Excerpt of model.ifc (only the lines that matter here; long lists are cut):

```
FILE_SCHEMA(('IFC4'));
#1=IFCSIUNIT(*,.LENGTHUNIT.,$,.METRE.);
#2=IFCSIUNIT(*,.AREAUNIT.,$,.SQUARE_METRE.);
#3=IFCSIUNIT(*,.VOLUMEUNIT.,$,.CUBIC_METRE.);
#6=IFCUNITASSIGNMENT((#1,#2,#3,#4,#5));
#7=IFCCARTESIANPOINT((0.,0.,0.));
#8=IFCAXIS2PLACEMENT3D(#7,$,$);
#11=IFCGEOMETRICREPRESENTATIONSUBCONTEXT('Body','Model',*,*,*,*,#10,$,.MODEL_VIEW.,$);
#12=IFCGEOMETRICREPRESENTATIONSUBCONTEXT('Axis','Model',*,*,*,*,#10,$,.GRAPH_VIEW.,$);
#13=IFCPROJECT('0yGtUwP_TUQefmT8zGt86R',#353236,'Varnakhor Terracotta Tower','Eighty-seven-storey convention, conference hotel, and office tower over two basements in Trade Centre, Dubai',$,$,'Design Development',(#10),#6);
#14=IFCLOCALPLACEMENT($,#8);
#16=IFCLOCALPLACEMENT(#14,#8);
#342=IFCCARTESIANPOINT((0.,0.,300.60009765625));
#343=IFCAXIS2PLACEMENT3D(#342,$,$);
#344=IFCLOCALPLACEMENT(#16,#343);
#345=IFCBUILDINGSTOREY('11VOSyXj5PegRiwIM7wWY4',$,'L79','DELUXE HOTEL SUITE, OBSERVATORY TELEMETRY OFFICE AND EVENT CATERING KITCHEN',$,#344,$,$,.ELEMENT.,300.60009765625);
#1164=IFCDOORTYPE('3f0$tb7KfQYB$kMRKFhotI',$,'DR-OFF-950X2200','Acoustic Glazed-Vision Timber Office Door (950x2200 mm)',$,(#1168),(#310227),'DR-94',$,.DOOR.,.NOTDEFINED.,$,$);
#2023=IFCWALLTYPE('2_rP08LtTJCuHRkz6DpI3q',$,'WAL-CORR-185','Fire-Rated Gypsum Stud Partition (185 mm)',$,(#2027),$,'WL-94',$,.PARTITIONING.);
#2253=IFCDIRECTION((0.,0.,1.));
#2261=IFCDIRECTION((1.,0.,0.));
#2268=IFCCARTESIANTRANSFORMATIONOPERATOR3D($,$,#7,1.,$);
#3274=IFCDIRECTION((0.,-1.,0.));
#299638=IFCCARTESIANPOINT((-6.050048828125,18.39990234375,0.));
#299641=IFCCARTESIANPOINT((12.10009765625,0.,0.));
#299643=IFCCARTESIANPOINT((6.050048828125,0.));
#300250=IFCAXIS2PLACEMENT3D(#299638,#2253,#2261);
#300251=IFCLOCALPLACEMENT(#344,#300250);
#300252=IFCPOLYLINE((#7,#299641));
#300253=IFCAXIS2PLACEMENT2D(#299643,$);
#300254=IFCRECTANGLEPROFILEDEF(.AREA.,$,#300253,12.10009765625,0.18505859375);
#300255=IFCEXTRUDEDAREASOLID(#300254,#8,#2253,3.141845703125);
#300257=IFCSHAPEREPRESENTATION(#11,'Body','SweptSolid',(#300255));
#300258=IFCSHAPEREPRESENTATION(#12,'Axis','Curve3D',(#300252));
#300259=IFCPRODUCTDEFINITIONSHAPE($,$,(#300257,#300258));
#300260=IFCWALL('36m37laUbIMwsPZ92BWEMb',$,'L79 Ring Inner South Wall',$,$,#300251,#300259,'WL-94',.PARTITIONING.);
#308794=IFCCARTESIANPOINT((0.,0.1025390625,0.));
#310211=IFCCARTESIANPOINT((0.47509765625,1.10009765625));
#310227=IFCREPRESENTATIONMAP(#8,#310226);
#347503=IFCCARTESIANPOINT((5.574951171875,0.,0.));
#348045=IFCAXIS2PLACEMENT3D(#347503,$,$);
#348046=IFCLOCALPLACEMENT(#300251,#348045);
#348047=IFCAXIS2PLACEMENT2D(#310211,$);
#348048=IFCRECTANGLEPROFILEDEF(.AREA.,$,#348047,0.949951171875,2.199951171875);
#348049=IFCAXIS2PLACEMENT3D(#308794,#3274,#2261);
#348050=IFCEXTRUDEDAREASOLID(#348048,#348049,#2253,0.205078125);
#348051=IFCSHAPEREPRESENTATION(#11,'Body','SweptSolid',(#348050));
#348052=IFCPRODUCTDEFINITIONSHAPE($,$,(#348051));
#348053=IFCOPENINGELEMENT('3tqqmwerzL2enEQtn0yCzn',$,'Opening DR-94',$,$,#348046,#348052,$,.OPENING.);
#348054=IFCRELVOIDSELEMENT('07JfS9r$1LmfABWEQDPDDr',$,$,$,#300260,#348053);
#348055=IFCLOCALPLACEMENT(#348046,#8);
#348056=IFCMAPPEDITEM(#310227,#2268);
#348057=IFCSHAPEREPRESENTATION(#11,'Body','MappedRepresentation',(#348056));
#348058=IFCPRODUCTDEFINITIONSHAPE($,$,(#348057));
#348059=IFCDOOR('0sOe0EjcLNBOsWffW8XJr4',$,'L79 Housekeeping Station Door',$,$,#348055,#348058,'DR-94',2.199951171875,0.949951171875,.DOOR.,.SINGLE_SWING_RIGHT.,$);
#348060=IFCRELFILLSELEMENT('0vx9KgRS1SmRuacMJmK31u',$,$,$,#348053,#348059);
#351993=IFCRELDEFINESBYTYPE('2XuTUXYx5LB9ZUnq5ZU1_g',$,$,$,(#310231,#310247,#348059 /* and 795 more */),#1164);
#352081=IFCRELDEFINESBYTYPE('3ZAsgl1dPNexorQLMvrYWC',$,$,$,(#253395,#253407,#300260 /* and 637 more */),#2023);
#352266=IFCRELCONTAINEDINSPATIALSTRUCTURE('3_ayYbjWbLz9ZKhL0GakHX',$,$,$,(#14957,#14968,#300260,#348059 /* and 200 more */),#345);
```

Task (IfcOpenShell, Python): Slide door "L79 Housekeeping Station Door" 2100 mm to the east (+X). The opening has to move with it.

```python
import ifcopenshell
import ifcopenshell.api.geometry
import ifcopenshell.util.placement

model = ifcopenshell.open("model.ifc")

door = model.by_guid("0sOe0EjcLNBOsWffW8XJr4")
opening = door.FillsVoids[0].RelatingOpeningElement
wall = opening.VoidsElements[0].RelatingBuildingElement

wall_matrix = ifcopenshell.util.placement.get_local_placement(wall.ObjectPlacement)
shift = wall_matrix[:3, 0] * 2.1
before = ifcopenshell.util.placement.get_local_placement(door.ObjectPlacement)[:3, 3].copy()

# The door is placed relative to its opening, so it follows when the opening moves.
matrix = ifcopenshell.util.placement.get_local_placement(opening.ObjectPlacement)
matrix[:3, 3] += shift
ifcopenshell.api.geometry.edit_object_placement(
    model, product=opening, matrix=matrix, is_si=False, should_transform_children=True
)

after = ifcopenshell.util.placement.get_local_placement(door.ObjectPlacement)[:3, 3]
print("door moved by", (after - before).round(3) + 0.0)

model.write("model-out.ifc")
```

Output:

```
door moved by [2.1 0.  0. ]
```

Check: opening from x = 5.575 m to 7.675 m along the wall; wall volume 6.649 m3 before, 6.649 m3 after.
